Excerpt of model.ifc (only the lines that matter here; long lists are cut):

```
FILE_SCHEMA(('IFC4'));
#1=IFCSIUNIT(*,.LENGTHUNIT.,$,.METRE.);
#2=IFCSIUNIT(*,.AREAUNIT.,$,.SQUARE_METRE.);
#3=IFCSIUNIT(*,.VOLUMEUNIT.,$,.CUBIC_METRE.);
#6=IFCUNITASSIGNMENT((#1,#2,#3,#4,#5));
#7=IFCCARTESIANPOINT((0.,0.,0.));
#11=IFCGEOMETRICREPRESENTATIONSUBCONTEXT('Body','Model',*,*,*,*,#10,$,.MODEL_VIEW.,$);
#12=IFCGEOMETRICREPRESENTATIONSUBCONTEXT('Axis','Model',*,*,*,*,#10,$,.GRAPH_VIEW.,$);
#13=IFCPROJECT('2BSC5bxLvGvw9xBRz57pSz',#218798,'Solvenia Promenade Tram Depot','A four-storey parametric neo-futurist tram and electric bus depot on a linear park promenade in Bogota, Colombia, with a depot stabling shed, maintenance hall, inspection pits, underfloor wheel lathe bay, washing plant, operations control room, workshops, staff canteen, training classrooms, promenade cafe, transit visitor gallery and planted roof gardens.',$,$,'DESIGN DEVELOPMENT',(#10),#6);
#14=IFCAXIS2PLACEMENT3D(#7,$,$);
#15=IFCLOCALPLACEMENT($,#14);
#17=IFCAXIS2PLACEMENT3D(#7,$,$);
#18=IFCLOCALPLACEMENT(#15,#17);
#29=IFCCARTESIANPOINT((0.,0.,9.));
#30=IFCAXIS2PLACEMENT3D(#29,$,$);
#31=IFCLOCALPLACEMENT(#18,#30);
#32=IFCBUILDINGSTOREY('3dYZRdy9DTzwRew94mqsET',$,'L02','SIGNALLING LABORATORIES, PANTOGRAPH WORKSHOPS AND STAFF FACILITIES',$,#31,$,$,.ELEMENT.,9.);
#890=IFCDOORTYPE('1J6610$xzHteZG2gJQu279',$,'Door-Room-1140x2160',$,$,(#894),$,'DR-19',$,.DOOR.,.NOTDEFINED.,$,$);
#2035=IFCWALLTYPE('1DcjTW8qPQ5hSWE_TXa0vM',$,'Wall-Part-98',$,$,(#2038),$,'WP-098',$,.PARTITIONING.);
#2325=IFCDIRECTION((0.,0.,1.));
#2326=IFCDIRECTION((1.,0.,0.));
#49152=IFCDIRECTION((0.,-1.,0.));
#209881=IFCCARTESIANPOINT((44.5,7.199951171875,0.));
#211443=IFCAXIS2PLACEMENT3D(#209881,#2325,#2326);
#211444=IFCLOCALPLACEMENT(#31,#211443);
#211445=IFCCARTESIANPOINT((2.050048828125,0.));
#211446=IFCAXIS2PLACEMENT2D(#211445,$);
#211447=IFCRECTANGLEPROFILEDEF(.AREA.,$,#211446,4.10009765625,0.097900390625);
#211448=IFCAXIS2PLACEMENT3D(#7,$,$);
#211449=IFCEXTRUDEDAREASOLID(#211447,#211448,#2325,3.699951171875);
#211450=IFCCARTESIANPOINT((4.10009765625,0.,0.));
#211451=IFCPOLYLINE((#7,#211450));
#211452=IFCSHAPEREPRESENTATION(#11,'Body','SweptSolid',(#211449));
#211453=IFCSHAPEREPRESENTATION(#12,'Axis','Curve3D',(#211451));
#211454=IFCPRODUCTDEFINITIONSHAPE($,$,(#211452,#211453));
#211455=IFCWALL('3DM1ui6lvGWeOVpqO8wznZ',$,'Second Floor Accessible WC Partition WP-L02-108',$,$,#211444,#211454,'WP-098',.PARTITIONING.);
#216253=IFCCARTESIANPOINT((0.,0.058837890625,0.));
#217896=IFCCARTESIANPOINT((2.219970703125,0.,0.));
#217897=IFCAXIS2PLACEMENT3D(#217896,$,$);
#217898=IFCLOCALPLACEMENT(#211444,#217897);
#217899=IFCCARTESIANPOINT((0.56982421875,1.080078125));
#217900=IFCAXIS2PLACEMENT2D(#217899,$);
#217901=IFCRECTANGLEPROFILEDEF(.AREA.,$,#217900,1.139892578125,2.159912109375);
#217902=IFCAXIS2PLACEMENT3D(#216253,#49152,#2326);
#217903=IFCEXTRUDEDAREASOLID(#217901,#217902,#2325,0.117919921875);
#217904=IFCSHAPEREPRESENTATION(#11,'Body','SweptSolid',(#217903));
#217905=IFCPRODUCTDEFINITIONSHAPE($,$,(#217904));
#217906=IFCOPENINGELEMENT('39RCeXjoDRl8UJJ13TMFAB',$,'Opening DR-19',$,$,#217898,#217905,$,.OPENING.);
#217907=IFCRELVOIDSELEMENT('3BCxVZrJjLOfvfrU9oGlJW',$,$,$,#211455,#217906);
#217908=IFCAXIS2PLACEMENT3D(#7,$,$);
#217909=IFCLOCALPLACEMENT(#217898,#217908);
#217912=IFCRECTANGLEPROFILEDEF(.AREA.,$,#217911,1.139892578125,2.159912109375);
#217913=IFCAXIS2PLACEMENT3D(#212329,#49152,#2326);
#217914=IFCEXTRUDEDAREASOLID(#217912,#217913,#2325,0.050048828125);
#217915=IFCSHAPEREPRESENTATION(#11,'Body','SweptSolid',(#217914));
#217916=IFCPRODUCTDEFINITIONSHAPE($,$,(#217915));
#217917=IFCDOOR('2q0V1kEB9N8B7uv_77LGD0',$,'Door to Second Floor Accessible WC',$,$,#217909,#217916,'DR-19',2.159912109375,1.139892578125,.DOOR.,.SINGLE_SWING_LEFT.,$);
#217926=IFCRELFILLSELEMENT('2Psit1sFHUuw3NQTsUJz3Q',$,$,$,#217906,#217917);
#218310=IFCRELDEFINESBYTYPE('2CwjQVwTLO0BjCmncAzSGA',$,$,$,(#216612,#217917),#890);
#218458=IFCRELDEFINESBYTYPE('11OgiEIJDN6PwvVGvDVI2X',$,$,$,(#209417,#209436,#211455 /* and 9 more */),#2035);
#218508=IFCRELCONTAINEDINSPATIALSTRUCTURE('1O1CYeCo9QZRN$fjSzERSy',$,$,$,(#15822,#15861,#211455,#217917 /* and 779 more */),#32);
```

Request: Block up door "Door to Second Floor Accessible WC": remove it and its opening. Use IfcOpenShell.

```python
import ifcopenshell
import ifcopenshell.api.feature
import ifcopenshell.api.root
import ifcopenshell.geom
import ifcopenshell.util.shape

model = ifcopenshell.open("model.ifc")
settings = ifcopenshell.geom.settings()


def volume(element):
    """Net volume in cubic metres, openings subtracted."""
    shape = ifcopenshell.geom.create_shape(settings, element)
    return ifcopenshell.util.shape.get_volume(shape.geometry)


door = model.by_id(217917)
opening = door.FillsVoids[0].RelatingOpeningElement
wall = opening.VoidsElements[0].RelatingBuildingElement
before = volume(wall)

ifcopenshell.api.root.remove_product(model, product=door)
ifcopenshell.api.feature.remove_feature(model, feature=opening)

after = volume(wall)

print(f"wall volume {before:.3f} -> {after:.3f} m3")

model.write("model_rev.ifc")
```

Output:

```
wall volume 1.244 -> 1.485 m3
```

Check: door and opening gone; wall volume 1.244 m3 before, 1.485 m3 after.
